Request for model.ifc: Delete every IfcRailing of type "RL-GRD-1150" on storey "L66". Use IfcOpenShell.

First a look at what the model holds.

```python
import ifcopenshell
import ifcopenshell.util.element

model = ifcopenshell.open("model.ifc")
print(model.schema)
storey = next(s for s in model.by_type("IfcBuildingStorey") if s.Name == "L66")
railings = [e for e in ifcopenshell.util.element.get_decomposition(storey) if e.is_a("IfcRailing")]
seen = {}
for e in railings:
    element_type = ifcopenshell.util.element.get_type(e)
    name = element_type.Name if element_type not in (None, e) else None
    seen[name] = seen.get(name, 0) + 1
for name, count in sorted(seen.items(), key=str):
    print(count, "x", name)
```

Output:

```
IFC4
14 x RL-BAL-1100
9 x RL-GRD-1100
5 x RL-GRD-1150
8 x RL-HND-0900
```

```python
import ifcopenshell
import ifcopenshell.api.root
import ifcopenshell.util.element

model = ifcopenshell.open("model.ifc")

storey = next(s for s in model.by_type("IfcBuildingStorey") if s.Name == "L66")
railings = [e for e in ifcopenshell.util.element.get_decomposition(storey) if e.is_a("IfcRailing")]
targets = [e for e in railings if (t := ifcopenshell.util.element.get_type(e)) not in (None, e) and t.Name == "RL-GRD-1150"]

for e in targets:
    ifcopenshell.api.root.remove_product(model, product=e)
print(len(targets), "removed")

model.write("model_v2.ifc")
```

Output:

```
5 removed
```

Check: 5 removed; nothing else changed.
